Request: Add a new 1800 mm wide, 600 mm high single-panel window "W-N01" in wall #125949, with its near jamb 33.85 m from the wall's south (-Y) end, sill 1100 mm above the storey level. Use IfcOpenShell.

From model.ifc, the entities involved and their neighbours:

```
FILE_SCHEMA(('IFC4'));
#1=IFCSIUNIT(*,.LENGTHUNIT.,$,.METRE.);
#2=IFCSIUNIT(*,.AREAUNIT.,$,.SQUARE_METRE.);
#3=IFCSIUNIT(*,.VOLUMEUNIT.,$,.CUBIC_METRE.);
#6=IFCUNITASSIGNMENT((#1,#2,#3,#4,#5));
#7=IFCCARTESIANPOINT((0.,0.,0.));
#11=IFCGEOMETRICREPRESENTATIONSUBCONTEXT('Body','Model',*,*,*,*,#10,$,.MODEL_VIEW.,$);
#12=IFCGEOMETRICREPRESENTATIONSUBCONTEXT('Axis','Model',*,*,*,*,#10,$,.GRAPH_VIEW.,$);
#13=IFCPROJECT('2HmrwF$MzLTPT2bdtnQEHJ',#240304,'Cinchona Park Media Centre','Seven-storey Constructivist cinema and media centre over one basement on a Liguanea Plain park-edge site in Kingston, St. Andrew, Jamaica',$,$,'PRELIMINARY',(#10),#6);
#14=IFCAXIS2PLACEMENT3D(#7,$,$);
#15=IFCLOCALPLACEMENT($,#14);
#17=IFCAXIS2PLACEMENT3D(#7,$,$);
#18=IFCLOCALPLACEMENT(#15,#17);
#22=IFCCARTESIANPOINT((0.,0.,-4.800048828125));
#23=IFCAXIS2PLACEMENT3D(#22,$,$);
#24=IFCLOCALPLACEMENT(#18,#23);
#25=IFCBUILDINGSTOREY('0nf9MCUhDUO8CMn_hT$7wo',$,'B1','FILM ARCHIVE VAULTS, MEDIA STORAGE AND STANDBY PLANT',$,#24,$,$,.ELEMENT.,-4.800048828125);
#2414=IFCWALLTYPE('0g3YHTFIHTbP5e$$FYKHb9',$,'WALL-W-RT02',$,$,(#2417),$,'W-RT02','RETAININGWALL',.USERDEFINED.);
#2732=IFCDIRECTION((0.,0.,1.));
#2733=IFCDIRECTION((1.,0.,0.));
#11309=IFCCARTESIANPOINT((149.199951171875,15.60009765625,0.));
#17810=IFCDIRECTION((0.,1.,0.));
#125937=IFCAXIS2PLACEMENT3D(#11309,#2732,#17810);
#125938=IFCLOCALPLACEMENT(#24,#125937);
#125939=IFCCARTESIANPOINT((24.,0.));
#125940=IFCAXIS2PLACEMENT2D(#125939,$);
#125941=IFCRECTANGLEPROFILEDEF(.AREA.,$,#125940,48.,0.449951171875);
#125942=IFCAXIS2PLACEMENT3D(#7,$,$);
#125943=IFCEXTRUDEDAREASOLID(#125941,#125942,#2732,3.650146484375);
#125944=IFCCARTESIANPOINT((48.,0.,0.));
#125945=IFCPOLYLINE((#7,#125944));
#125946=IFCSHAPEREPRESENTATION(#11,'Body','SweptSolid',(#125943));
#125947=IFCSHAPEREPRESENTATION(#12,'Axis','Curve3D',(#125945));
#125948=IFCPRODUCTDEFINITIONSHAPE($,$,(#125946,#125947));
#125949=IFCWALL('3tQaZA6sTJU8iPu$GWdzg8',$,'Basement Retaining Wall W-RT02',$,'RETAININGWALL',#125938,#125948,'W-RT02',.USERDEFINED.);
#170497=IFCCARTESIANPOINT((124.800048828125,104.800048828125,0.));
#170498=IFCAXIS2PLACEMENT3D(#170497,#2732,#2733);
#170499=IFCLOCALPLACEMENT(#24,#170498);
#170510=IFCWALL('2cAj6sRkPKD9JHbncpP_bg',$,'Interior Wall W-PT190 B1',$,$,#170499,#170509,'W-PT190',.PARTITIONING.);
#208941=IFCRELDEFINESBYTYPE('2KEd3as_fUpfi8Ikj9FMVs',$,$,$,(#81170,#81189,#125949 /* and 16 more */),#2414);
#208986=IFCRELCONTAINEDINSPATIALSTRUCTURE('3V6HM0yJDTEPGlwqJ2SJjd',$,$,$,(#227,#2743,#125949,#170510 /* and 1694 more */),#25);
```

```python
import numpy as np
import ifcopenshell
import ifcopenshell.api.feature
import ifcopenshell.api.geometry
import ifcopenshell.api.root
import ifcopenshell.api.spatial
import ifcopenshell.geom
import ifcopenshell.util.element
import ifcopenshell.util.placement
import ifcopenshell.util.representation
import ifcopenshell.util.shape
import ifcopenshell.util.unit

model = ifcopenshell.open("model.ifc")
unit_scale = ifcopenshell.util.unit.calculate_unit_scale(model)
settings = ifcopenshell.geom.settings()


def volume(element):
    """Net volume in cubic metres, openings subtracted."""
    shape = ifcopenshell.geom.create_shape(settings, element)
    return ifcopenshell.util.shape.get_volume(shape.geometry)


wall = model.by_guid("3tQaZA6sTJU8iPu$GWdzg8")
storey = ifcopenshell.util.element.get_container(wall, ifc_class="IfcBuildingStorey")
context = ifcopenshell.util.representation.get_context(model, "Model", "Body", "MODEL_VIEW")
before = volume(wall)

width, height, from_end, sill = 1.8, 0.6, 33.85, 1.1  # metres

# The wall runs along its own X axis, and the end named is its -X end.
wall_shape = ifcopenshell.geom.create_shape(settings, wall)
x, y, z = ifcopenshell.util.shape.get_vertices(wall_shape.geometry).T
start = x.min() + from_end
face, thickness = float(y.min()), float(y.max() - y.min())
wall_matrix = ifcopenshell.util.placement.get_local_placement(wall.ObjectPlacement)
level = ifcopenshell.util.placement.get_local_placement(storey.ObjectPlacement)[2, 3]


def in_wall(x, y):
    """Placement at x, y metres in the wall's axes, at sill height."""
    matrix = wall_matrix.copy()
    matrix[:, 3] = wall_matrix @ np.array([x / unit_scale, y / unit_scale, 0.0, 1.0])
    matrix[2, 3] = level + sill / unit_scale
    return matrix


# Opening: a box that overshoots both wall faces by 50 mm.
opening = ifcopenshell.api.root.create_entity(model, ifc_class="IfcOpeningElement", predefined_type="OPENING")
box = ifcopenshell.api.geometry.add_wall_representation(
    model, context=context, length=width, height=height, thickness=thickness + 0.1
)
ifcopenshell.api.geometry.assign_representation(model, product=opening, representation=box)
ifcopenshell.api.geometry.edit_object_placement(model, product=opening, matrix=in_wall(start, face - 0.05), is_si=False)
ifcopenshell.api.feature.add_feature(model, feature=opening, element=wall)

window = ifcopenshell.api.root.create_entity(model, ifc_class="IfcWindow", name="W-N01", predefined_type="WINDOW")
window.OverallWidth, window.OverallHeight = width / unit_scale, height / unit_scale
window.PartitioningType = "SINGLE_PANEL"
body = ifcopenshell.api.geometry.add_window_representation(
    model,
    context=context,
    overall_width=window.OverallWidth,
    overall_height=window.OverallHeight,
    partition_type="SINGLE_PANEL",
)
ifcopenshell.api.geometry.assign_representation(model, product=window, representation=body)
ifcopenshell.api.spatial.assign_container(model, products=[window], relating_structure=storey)
ifcopenshell.api.feature.add_filling(model, opening=opening, element=window)

# Centre the window in the wall's thickness.
ifcopenshell.api.geometry.edit_object_placement(model, product=window, matrix=in_wall(start, face), is_si=False)
window_shape = ifcopenshell.geom.create_shape(settings, window)
depth = ifcopenshell.util.shape.get_vertices(window_shape.geometry)[:, 1]
offset = face + thickness / 2 - (depth.min() + depth.max()) / 2
ifcopenshell.api.geometry.edit_object_placement(model, product=window, matrix=in_wall(start, offset), is_si=False)

after = volume(wall)

print(f"wall volume {before:.3f} -> {after:.3f} m3")

model.write("model_rev.ifc")
```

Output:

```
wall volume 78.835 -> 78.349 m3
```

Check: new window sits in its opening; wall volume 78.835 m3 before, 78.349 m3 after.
